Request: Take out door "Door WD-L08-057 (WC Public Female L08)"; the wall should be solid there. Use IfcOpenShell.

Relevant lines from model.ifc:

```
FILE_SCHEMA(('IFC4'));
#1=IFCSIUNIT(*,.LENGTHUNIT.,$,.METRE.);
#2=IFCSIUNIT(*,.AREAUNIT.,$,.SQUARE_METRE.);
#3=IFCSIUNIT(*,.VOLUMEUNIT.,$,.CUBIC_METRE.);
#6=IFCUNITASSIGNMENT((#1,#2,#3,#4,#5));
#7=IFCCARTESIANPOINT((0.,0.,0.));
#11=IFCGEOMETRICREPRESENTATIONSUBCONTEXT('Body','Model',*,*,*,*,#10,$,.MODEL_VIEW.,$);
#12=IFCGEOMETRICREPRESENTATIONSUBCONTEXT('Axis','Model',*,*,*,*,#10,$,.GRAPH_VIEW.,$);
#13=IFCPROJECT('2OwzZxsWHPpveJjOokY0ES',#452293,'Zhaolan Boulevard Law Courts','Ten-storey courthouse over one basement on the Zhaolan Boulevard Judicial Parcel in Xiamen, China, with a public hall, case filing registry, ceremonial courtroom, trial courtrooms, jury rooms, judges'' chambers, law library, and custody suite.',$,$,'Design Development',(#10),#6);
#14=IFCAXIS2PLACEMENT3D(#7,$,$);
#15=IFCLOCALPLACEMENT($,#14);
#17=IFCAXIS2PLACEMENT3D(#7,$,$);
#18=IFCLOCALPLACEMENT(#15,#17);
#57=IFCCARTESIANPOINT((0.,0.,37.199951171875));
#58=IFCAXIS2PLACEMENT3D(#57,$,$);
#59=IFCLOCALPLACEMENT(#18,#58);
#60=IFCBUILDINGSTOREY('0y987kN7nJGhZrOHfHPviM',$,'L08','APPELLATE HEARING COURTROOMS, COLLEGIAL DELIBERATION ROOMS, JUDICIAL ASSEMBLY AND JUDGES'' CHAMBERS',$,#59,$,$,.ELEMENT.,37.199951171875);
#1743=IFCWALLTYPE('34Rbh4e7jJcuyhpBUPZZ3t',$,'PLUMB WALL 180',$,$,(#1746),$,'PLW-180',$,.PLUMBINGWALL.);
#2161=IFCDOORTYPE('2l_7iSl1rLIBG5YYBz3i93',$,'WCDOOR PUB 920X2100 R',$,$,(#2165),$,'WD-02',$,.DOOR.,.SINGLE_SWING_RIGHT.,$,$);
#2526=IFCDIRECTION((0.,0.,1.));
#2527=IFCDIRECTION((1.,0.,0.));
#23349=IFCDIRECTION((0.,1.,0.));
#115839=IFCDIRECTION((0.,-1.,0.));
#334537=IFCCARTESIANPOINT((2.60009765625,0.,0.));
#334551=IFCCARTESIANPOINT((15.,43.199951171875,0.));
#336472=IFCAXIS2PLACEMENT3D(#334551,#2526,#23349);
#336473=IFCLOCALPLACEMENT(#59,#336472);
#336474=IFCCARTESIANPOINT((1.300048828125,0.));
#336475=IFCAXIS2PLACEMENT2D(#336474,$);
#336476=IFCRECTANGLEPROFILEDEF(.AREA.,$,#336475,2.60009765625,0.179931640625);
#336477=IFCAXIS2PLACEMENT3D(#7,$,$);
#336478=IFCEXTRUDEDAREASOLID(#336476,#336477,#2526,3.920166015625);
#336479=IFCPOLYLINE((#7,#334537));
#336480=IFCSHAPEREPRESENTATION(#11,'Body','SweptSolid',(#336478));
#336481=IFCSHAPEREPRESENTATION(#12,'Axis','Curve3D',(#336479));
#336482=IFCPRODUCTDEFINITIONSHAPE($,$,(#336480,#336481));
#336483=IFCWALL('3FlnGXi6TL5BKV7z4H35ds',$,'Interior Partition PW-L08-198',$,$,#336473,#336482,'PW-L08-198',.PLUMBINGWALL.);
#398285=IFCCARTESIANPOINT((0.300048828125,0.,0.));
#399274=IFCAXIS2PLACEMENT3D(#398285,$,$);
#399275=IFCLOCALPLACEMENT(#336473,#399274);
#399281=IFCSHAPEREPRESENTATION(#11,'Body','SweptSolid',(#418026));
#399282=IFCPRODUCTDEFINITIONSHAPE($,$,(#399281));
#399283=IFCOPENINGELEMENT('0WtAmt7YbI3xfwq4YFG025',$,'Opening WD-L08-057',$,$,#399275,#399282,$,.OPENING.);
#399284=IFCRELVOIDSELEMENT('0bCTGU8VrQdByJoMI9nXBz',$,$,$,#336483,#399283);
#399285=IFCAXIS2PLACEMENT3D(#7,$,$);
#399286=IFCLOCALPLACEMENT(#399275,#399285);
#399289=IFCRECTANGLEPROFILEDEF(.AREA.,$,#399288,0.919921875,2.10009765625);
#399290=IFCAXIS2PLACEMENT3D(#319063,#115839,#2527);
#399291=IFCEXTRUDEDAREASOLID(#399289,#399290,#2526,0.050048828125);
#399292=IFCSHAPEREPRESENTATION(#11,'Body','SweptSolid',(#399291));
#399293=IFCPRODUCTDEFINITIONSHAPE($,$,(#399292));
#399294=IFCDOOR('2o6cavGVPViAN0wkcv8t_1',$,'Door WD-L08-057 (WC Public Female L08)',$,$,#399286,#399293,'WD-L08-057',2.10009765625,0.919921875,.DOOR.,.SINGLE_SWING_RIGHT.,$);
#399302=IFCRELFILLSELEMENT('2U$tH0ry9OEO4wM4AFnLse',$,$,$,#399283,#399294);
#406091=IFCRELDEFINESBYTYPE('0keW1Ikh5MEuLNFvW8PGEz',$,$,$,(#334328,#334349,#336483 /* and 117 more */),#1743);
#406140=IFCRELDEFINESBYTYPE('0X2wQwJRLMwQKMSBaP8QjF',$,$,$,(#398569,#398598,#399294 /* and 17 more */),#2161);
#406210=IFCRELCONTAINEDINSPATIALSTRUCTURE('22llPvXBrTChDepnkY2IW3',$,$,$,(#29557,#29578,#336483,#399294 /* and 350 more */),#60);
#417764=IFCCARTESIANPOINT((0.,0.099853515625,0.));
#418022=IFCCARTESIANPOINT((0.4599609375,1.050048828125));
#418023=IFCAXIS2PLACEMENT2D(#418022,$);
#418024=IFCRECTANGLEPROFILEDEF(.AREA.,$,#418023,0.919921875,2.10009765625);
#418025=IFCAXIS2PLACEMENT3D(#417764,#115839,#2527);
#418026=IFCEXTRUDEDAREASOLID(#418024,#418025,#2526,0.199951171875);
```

```python
import ifcopenshell
import ifcopenshell.api.feature
import ifcopenshell.api.root
import ifcopenshell.geom
import ifcopenshell.util.shape

model = ifcopenshell.open("model.ifc")
settings = ifcopenshell.geom.settings()


def volume(element):
    """Net volume in cubic metres, openings subtracted."""
    shape = ifcopenshell.geom.create_shape(settings, element)
    return ifcopenshell.util.shape.get_volume(shape.geometry)


door = model.by_guid("2o6cavGVPViAN0wkcv8t_1")
opening = door.FillsVoids[0].RelatingOpeningElement
wall = opening.VoidsElements[0].RelatingBuildingElement
before = volume(wall)

ifcopenshell.api.root.remove_product(model, product=door)
ifcopenshell.api.feature.remove_feature(model, feature=opening)

after = volume(wall)

print(f"wall volume {before:.3f} -> {after:.3f} m3")

model.write("model_edited.ifc")
```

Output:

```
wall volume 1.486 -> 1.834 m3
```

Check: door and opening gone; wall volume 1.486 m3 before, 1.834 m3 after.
